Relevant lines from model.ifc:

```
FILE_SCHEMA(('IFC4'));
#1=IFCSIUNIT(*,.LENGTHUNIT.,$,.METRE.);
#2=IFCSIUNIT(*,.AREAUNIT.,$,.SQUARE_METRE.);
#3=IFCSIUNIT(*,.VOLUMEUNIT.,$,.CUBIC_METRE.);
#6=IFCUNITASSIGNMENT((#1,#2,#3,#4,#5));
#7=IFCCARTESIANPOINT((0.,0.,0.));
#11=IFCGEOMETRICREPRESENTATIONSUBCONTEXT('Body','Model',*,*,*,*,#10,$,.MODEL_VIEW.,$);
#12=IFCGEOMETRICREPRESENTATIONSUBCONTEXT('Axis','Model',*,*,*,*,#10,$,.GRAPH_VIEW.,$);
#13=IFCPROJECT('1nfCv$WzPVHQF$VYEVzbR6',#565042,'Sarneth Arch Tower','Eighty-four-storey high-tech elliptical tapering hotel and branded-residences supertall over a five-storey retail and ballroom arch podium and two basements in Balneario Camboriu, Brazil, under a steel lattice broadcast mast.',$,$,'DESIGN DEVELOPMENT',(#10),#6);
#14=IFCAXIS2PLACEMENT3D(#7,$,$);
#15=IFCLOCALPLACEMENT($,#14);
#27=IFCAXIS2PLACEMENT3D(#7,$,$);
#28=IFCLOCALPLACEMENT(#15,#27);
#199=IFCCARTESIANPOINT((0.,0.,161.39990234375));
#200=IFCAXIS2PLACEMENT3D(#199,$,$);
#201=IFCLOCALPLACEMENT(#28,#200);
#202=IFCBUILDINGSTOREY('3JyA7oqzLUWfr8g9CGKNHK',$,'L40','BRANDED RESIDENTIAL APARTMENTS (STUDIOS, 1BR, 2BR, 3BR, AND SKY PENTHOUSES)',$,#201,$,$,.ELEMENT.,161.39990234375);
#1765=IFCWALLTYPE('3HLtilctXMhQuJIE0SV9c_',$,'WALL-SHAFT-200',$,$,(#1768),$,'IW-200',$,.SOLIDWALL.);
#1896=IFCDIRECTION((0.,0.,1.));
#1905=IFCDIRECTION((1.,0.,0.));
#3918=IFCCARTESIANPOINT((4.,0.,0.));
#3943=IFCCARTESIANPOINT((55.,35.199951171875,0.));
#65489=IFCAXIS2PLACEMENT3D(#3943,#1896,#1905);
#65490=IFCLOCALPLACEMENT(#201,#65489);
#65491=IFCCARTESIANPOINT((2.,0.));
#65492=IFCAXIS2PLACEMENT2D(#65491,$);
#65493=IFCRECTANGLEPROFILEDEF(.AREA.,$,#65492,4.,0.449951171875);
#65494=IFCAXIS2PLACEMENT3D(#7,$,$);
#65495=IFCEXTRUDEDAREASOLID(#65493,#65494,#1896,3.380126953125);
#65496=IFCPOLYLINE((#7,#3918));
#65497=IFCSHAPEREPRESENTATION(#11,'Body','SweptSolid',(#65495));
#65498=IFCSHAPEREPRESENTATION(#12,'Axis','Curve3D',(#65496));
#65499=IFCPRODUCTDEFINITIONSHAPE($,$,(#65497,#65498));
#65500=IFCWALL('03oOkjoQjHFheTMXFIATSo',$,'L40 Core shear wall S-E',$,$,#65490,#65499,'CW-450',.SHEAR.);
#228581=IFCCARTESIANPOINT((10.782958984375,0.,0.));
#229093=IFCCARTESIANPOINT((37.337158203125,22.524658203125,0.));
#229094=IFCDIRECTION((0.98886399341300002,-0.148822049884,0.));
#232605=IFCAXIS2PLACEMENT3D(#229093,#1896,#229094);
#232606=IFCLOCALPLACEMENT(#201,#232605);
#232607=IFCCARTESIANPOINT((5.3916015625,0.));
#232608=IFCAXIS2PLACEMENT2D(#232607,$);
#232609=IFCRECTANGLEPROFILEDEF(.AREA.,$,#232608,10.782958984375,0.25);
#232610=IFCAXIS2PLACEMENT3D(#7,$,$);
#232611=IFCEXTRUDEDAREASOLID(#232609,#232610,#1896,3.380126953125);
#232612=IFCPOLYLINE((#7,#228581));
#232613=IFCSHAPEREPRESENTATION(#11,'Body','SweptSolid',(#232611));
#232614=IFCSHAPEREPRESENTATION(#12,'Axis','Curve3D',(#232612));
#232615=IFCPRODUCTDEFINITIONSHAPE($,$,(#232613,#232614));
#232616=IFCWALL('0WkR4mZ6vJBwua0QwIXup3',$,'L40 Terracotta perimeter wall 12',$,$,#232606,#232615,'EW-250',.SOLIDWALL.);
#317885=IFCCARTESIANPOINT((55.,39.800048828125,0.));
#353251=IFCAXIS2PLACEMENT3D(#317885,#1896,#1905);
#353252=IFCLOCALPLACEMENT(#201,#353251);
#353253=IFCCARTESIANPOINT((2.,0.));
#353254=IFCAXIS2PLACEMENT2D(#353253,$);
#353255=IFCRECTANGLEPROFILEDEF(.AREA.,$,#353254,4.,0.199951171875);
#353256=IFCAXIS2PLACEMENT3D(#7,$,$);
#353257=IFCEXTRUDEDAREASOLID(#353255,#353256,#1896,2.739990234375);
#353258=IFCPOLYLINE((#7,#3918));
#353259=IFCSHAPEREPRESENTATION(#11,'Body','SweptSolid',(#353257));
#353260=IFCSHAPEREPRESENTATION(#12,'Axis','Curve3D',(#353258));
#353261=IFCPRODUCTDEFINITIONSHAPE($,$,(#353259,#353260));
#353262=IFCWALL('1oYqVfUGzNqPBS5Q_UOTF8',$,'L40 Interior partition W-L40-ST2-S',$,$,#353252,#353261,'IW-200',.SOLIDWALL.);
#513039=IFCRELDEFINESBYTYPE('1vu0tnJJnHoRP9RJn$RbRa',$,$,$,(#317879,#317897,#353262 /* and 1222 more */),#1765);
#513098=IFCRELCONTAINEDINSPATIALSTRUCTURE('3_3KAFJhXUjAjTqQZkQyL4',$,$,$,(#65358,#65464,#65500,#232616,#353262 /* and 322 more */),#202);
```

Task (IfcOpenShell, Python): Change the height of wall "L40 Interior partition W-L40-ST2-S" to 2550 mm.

```python
import ifcopenshell
import ifcopenshell.geom
import ifcopenshell.util.representation
import ifcopenshell.util.shape
import ifcopenshell.util.unit

model = ifcopenshell.open("model.ifc")
unit_scale = ifcopenshell.util.unit.calculate_unit_scale(model)
settings = ifcopenshell.geom.settings()


def volume(element):
    """Net volume in cubic metres, openings subtracted."""
    shape = ifcopenshell.geom.create_shape(settings, element)
    return ifcopenshell.util.shape.get_volume(shape.geometry)


wall = model.by_guid("1oYqVfUGzNqPBS5Q_UOTF8")
before = volume(wall)

body = ifcopenshell.util.representation.get_representation(wall, "Model", "Body")
solid = body.Items[0]
old_height = solid.Depth
solid.Depth = 2.55 / unit_scale
after = volume(wall)

print(f"height {old_height:g} -> {solid.Depth:g}, volume {before:.3f} -> {after:.3f} m3")

model.write("model_v2.ifc")
```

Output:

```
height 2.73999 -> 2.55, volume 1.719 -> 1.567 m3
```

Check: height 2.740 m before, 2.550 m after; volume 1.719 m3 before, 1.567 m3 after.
